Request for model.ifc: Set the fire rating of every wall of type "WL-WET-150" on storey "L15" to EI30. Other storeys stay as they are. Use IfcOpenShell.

First a look at what the model holds.

```python
import ifcopenshell
import ifcopenshell.util.element

model = ifcopenshell.open("model.ifc")
print(model.schema)
storey = next(s for s in model.by_type("IfcBuildingStorey") if s.Name == "L15")
walls = [e for e in ifcopenshell.util.element.get_decomposition(storey) if e.is_a("IfcWall")]
seen = {}
for e in walls:
    element_type = ifcopenshell.util.element.get_type(e)
    key = (element_type.Name if element_type != e and element_type else None, ifcopenshell.util.element.get_pset(e, "Pset_WallCommon", "FireRating"))
    seen[key] = seen.get(key, 0) + 1
for (name, value), count in sorted(seen.items(), key=str):
    print(count, "x", name, "|", value)
```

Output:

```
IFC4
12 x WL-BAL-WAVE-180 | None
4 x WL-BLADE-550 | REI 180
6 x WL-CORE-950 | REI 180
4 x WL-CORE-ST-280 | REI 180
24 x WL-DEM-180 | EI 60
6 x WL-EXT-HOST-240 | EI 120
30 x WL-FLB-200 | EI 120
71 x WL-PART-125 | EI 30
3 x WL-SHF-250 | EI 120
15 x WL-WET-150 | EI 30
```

```python
import ifcopenshell
import ifcopenshell.api.pset
import ifcopenshell.util.element

model = ifcopenshell.open("model.ifc")

storey = next(s for s in model.by_type("IfcBuildingStorey") if s.Name == "L15")
walls = [e for e in ifcopenshell.util.element.get_decomposition(storey) if e.is_a("IfcWall")]

count = 0
for e in walls:
    element_type = ifcopenshell.util.element.get_type(e)
    if element_type in (None, e) or element_type.Name != "WL-WET-150":
        continue
    found = ifcopenshell.util.element.get_pset(e, "Pset_WallCommon", should_inherit=False)
    if found:
        pset = model.by_id(found["id"])
        if len(ifcopenshell.util.element.get_elements_by_pset(pset)) > 1:
            pset = ifcopenshell.api.pset.unshare_pset(model, products=[e], pset=pset)[0]
    else:
        pset = ifcopenshell.api.pset.add_pset(model, product=e, name="Pset_WallCommon")
    ifcopenshell.api.pset.edit_pset(model, pset=pset, properties={"FireRating": "EI30"})
    count += 1

print(count, "walls updated")

model.write("model_updated.ifc")
```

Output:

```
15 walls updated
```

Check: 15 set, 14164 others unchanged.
